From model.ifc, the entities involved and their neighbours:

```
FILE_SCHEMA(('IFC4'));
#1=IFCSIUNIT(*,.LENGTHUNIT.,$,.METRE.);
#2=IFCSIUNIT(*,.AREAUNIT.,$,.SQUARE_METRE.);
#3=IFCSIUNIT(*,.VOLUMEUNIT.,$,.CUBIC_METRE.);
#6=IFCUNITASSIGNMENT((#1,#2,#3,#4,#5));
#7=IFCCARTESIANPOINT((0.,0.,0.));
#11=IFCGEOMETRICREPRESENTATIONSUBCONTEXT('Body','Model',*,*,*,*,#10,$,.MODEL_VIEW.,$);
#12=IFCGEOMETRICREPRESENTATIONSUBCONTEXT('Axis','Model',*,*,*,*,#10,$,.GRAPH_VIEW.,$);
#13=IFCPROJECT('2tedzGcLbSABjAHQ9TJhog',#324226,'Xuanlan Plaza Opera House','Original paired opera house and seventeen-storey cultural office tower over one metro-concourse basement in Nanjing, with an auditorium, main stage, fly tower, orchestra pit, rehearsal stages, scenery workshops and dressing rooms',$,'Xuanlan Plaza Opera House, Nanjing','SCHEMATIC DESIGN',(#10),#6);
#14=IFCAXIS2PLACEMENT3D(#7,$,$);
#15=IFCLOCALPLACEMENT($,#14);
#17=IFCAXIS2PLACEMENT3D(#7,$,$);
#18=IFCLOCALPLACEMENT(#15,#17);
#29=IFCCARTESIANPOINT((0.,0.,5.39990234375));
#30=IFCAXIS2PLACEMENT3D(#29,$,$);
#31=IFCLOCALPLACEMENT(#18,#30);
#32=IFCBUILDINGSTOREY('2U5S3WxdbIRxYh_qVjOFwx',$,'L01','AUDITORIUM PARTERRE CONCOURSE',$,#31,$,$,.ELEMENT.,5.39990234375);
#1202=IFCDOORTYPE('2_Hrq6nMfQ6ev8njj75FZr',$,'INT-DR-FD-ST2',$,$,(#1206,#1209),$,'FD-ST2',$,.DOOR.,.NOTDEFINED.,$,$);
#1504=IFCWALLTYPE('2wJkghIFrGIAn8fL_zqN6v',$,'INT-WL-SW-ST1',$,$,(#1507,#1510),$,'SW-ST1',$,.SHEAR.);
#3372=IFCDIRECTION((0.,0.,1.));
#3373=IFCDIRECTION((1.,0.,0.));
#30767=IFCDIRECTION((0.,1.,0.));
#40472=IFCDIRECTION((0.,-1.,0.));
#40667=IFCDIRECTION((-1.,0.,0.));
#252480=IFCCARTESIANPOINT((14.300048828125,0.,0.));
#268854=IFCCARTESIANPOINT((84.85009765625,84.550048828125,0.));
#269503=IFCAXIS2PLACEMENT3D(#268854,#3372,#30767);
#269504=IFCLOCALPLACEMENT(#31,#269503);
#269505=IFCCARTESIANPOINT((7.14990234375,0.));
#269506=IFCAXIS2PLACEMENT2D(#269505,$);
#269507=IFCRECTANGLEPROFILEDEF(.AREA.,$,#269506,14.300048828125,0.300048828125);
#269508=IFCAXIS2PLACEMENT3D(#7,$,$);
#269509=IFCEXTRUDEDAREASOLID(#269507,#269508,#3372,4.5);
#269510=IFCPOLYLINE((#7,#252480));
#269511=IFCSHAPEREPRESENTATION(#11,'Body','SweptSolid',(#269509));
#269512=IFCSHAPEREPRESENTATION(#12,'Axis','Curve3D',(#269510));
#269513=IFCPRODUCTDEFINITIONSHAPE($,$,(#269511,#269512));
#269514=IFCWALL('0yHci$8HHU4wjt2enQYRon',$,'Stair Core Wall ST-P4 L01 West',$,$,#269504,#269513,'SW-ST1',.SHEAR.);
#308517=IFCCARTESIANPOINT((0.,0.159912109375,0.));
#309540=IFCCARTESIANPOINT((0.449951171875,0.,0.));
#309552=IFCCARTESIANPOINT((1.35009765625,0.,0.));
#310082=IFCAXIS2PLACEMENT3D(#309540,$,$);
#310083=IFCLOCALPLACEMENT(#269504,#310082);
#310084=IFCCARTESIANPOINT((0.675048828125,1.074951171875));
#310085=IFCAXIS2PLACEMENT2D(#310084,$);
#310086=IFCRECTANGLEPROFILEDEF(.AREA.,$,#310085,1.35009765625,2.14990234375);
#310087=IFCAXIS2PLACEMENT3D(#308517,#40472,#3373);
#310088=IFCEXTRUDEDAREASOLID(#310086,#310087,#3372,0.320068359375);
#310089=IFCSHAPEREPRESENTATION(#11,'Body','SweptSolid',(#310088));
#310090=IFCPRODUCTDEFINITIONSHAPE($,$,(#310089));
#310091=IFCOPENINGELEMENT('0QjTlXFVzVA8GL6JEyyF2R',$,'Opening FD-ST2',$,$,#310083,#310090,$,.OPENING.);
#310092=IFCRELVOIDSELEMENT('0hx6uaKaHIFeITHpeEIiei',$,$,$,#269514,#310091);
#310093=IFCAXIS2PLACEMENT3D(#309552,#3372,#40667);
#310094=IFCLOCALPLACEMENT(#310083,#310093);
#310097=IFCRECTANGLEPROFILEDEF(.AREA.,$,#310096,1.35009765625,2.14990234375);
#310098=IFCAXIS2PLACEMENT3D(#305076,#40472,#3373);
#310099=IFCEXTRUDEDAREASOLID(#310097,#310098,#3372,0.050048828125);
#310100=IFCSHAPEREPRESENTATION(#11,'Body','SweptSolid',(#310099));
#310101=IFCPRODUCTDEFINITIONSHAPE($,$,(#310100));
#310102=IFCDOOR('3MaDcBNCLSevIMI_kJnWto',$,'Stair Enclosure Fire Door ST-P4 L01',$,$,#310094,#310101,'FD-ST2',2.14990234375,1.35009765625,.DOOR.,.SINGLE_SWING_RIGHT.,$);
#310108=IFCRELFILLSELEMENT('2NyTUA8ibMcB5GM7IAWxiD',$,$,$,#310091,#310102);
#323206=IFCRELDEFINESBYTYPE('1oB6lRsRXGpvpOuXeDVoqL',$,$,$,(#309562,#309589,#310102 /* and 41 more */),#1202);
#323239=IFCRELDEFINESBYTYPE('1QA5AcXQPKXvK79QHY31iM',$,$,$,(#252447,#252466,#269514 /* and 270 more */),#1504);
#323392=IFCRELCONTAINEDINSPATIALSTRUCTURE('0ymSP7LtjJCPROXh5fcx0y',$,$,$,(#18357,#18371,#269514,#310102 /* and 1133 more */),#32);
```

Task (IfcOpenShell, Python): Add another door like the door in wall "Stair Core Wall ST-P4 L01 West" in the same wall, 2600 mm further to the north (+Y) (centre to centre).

```python
import ifcopenshell
import ifcopenshell.api.feature
import ifcopenshell.api.geometry
import ifcopenshell.api.root
import ifcopenshell.geom
import ifcopenshell.util.element
import ifcopenshell.util.placement
import ifcopenshell.util.shape

model = ifcopenshell.open("model.ifc")
settings = ifcopenshell.geom.settings()


def volume(element):
    """Net volume in cubic metres, openings subtracted."""
    shape = ifcopenshell.geom.create_shape(settings, element)
    return ifcopenshell.util.shape.get_volume(shape.geometry)


door = model.by_guid("3MaDcBNCLSevIMI_kJnWto")
opening = door.FillsVoids[0].RelatingOpeningElement
wall = opening.VoidsElements[0].RelatingBuildingElement
before = volume(wall)
shift = ifcopenshell.util.placement.get_local_placement(wall.ObjectPlacement)[:3, 0] * 2.6

# copy_class copies the void relationship, type, container and properties, but no geometry.
new_opening = ifcopenshell.api.root.copy_class(model, product=opening)
new_opening.Representation = ifcopenshell.util.element.copy_deep(
    model, opening.Representation, exclude=["IfcGeometricRepresentationContext", "IfcRepresentationMap"]
)
new_door = ifcopenshell.api.root.copy_class(model, product=door)
new_door.Representation = ifcopenshell.util.element.copy_deep(
    model, door.Representation, exclude=["IfcGeometricRepresentationContext", "IfcRepresentationMap"]
)
new_door.Tag = None
ifcopenshell.api.feature.add_filling(model, opening=new_opening, element=new_door)

for old, new in ((opening, new_opening), (door, new_door)):
    matrix = ifcopenshell.util.placement.get_local_placement(old.ObjectPlacement)
    matrix[:3, 3] += shift
    ifcopenshell.api.geometry.edit_object_placement(model, product=new, matrix=matrix, is_si=False)

after = volume(wall)

print(f"wall volume {before:.3f} -> {after:.3f} m3")

model.write("model_updated.ifc")
```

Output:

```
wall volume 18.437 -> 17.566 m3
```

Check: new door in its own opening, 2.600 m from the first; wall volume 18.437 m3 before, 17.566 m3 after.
